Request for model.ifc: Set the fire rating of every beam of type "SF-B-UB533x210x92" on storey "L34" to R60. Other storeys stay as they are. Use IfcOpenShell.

First a look at what the model holds.

```python
import ifcopenshell
import ifcopenshell.util.element

model = ifcopenshell.open("model.ifc")
print(model.schema)
storey = next(s for s in model.by_type("IfcBuildingStorey") if s.Name == "L34")
beams = [e for e in ifcopenshell.util.element.get_decomposition(storey) if e.is_a("IfcBeam")]
seen = {}
for e in beams:
    element_type = ifcopenshell.util.element.get_type(e)
    key = (element_type.Name if element_type != e and element_type else None, ifcopenshell.util.element.get_pset(e, "Pset_BeamCommon", "FireRating"))
    seen[key] = seen.get(key, 0) + 1
for (name, value), count in sorted(seen.items(), key=str):
    print(count, "x", name, "|", value)
```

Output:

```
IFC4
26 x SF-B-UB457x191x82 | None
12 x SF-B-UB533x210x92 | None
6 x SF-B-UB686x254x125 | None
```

```python
import ifcopenshell
import ifcopenshell.api.pset
import ifcopenshell.util.element

model = ifcopenshell.open("model.ifc")

storey = next(s for s in model.by_type("IfcBuildingStorey") if s.Name == "L34")
beams = [e for e in ifcopenshell.util.element.get_decomposition(storey) if e.is_a("IfcBeam")]

count = 0
for e in beams:
    element_type = ifcopenshell.util.element.get_type(e)
    if element_type in (None, e) or element_type.Name != "SF-B-UB533x210x92":
        continue
    found = ifcopenshell.util.element.get_pset(e, "Pset_BeamCommon", should_inherit=False)
    if found:
        pset = model.by_id(found["id"])
        if len(ifcopenshell.util.element.get_elements_by_pset(pset)) > 1:
            pset = ifcopenshell.api.pset.unshare_pset(model, products=[e], pset=pset)[0]
    else:
        pset = ifcopenshell.api.pset.add_pset(model, product=e, name="Pset_BeamCommon")
    ifcopenshell.api.pset.edit_pset(model, pset=pset, properties={"FireRating": "R60"})
    count += 1

print(count, "beams updated")

model.write("model-out.ifc")
```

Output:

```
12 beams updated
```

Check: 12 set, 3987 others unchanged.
